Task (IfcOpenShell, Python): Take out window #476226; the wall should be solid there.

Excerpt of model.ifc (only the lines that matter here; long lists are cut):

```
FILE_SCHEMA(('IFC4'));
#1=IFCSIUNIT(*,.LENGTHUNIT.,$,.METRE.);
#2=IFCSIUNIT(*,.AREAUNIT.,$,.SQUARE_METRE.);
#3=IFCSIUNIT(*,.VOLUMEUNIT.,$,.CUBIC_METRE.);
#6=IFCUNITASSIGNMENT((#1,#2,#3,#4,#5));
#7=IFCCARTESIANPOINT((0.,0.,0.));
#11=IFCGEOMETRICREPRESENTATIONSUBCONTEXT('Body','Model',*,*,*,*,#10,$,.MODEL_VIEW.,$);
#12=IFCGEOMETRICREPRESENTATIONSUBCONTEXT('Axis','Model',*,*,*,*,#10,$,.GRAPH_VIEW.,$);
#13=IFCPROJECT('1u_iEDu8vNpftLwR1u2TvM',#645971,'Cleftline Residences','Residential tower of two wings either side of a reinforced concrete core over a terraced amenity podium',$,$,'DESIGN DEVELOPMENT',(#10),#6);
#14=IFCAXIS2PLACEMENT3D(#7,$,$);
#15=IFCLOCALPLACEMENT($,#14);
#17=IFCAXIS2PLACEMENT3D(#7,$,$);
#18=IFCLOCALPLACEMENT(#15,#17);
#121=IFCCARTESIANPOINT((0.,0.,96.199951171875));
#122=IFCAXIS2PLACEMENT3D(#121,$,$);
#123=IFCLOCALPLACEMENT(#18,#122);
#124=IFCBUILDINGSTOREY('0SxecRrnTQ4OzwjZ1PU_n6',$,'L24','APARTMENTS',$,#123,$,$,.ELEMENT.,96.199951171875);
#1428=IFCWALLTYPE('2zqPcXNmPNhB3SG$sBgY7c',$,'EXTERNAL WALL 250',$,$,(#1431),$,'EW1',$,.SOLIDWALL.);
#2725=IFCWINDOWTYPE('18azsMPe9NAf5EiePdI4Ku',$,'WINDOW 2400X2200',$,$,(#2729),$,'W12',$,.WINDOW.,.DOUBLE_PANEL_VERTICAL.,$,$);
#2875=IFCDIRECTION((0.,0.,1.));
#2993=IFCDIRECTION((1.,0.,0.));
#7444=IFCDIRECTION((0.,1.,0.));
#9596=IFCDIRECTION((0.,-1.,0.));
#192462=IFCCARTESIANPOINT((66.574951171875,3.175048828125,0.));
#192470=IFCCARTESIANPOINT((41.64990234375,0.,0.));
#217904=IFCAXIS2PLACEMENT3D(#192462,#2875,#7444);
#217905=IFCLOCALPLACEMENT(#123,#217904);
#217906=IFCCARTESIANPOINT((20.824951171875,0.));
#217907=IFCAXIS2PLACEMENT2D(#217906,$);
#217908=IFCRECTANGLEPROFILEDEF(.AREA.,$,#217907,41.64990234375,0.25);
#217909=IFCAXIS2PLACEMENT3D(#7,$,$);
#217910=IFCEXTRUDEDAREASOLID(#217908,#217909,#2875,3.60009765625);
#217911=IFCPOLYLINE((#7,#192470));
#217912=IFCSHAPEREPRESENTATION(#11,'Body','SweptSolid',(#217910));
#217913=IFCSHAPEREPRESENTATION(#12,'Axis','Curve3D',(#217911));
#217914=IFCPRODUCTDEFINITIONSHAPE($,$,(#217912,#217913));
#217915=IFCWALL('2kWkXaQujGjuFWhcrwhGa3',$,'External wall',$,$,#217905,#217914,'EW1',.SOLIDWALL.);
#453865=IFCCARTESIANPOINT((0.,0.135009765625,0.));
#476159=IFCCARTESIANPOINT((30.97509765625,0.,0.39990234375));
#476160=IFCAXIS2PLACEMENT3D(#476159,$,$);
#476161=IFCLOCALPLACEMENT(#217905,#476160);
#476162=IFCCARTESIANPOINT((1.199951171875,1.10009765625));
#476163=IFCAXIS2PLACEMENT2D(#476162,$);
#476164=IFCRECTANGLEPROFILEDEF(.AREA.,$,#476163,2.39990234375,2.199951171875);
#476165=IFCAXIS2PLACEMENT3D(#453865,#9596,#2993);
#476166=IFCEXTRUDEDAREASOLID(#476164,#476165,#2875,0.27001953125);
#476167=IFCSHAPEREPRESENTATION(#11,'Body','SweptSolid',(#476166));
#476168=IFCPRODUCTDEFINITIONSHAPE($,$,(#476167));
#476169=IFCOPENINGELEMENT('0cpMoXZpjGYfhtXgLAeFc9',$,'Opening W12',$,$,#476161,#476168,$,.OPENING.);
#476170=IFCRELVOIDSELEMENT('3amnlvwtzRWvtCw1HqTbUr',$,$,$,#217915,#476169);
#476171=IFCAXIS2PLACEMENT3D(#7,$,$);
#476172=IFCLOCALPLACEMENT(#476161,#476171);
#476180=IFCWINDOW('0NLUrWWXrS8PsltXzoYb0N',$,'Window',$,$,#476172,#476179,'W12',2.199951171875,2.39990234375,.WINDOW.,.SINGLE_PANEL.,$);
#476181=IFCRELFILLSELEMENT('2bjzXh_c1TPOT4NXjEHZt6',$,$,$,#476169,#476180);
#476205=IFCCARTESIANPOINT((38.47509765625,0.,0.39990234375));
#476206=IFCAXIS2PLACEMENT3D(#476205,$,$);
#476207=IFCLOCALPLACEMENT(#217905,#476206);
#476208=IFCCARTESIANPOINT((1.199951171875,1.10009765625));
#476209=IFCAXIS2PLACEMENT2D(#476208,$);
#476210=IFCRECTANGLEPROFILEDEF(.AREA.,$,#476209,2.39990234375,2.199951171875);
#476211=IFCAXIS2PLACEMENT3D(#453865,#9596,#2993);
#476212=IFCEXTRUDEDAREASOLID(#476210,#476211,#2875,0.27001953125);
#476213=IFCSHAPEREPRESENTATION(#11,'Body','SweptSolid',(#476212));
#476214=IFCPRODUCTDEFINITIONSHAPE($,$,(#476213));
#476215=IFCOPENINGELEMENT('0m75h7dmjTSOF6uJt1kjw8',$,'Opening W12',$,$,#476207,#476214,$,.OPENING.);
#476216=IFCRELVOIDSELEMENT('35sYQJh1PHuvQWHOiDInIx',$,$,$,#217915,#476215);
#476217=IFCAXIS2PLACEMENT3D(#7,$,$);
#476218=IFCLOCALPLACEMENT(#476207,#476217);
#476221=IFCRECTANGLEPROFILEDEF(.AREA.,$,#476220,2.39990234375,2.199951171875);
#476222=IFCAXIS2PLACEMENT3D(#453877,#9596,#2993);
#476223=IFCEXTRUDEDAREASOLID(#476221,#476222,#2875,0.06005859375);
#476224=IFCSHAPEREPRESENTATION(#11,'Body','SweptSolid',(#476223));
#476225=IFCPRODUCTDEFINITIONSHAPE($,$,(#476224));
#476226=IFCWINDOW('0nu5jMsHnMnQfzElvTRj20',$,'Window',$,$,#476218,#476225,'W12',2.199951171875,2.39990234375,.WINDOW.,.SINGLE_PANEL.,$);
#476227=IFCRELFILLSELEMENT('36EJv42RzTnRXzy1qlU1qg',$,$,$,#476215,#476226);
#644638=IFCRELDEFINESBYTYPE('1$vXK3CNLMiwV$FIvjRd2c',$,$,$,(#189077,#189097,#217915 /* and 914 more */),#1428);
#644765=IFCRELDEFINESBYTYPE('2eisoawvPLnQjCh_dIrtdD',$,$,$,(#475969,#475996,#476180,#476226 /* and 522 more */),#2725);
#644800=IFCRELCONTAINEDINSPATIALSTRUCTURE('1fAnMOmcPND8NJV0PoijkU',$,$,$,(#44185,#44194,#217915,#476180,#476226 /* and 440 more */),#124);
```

```python
import ifcopenshell
import ifcopenshell.api.feature
import ifcopenshell.api.root
import ifcopenshell.geom
import ifcopenshell.util.shape

model = ifcopenshell.open("model.ifc")
settings = ifcopenshell.geom.settings()


def volume(element):
    """Net volume in cubic metres, openings subtracted."""
    shape = ifcopenshell.geom.create_shape(settings, element)
    return ifcopenshell.util.shape.get_volume(shape.geometry)


window = model.by_guid("0nu5jMsHnMnQfzElvTRj20")
opening = window.FillsVoids[0].RelatingOpeningElement
wall = opening.VoidsElements[0].RelatingBuildingElement
before = volume(wall)

ifcopenshell.api.root.remove_product(model, product=window)
ifcopenshell.api.feature.remove_feature(model, feature=opening)

after = volume(wall)

print(f"wall volume {before:.3f} -> {after:.3f} m3")

model.write("model_updated.ifc")
```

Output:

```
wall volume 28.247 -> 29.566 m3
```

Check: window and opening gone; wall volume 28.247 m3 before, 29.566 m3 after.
